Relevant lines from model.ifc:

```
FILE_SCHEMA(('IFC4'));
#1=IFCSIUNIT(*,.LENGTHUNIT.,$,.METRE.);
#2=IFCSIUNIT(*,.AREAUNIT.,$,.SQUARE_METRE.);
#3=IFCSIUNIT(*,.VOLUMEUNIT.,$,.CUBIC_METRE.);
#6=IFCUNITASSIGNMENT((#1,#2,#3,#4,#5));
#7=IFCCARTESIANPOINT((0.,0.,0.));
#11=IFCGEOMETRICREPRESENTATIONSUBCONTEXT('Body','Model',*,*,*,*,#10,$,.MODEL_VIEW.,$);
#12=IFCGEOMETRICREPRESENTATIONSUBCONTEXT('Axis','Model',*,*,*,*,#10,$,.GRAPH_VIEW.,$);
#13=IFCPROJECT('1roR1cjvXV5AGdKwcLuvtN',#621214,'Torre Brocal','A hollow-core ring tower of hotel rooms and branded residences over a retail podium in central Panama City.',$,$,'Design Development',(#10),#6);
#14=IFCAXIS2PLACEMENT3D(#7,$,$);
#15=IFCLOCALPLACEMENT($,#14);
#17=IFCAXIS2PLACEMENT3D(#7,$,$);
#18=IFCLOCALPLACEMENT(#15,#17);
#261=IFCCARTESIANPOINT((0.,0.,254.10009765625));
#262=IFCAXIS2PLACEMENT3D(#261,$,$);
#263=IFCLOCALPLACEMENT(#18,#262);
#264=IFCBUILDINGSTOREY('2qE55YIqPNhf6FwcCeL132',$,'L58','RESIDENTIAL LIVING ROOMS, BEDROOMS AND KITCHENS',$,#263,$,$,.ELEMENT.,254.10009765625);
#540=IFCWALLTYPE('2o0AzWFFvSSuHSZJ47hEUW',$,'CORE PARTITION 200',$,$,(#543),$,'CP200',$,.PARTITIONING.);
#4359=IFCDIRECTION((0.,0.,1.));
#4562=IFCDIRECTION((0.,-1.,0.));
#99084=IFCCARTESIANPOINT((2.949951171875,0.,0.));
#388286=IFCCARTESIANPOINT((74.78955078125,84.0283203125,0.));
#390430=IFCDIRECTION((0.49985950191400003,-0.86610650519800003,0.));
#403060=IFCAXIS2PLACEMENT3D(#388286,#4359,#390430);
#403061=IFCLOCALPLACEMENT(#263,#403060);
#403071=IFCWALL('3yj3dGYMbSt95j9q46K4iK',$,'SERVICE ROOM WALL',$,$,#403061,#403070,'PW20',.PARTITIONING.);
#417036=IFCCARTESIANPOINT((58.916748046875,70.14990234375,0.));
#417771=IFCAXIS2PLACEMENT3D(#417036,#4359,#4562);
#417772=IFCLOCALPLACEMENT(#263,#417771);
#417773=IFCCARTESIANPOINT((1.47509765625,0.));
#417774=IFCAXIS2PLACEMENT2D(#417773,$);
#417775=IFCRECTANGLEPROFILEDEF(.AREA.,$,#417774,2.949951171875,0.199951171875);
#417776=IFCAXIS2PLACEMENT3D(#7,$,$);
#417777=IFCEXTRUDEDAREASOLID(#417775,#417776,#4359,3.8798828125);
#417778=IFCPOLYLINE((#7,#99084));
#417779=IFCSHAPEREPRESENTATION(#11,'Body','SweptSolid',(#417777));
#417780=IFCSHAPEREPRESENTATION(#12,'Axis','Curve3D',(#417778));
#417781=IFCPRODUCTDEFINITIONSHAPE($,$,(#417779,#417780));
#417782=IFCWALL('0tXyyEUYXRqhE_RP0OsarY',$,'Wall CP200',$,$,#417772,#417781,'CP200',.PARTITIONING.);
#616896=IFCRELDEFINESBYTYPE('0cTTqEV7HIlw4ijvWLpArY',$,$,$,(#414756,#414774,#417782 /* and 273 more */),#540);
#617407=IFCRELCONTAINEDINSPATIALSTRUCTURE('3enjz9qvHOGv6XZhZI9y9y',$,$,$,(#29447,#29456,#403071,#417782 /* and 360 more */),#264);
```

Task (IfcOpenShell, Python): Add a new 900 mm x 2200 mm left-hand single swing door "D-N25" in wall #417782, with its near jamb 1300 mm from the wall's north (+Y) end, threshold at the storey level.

```python
import numpy as np
import ifcopenshell
import ifcopenshell.api.feature
import ifcopenshell.api.geometry
import ifcopenshell.api.root
import ifcopenshell.api.spatial
import ifcopenshell.geom
import ifcopenshell.util.element
import ifcopenshell.util.placement
import ifcopenshell.util.representation
import ifcopenshell.util.shape
import ifcopenshell.util.unit

model = ifcopenshell.open("model.ifc")
unit_scale = ifcopenshell.util.unit.calculate_unit_scale(model)
settings = ifcopenshell.geom.settings()


def volume(element):
    """Net volume in cubic metres, openings subtracted."""
    shape = ifcopenshell.geom.create_shape(settings, element)
    return ifcopenshell.util.shape.get_volume(shape.geometry)


wall = model.by_guid("0tXyyEUYXRqhE_RP0OsarY")
storey = ifcopenshell.util.element.get_container(wall, ifc_class="IfcBuildingStorey")
context = ifcopenshell.util.representation.get_context(model, "Model", "Body", "MODEL_VIEW")
before = volume(wall)

width, height, from_end, sill = 0.9, 2.2, 1.3, 0.0  # metres

# The wall runs along its own X axis, and the end named is its -X end.
wall_shape = ifcopenshell.geom.create_shape(settings, wall)
x, y, z = ifcopenshell.util.shape.get_vertices(wall_shape.geometry).T
start = x.min() + from_end
face, thickness = float(y.min()), float(y.max() - y.min())
wall_matrix = ifcopenshell.util.placement.get_local_placement(wall.ObjectPlacement)
level = ifcopenshell.util.placement.get_local_placement(storey.ObjectPlacement)[2, 3]


def in_wall(x, y):
    """Placement at x, y metres in the wall's axes, at sill height."""
    matrix = wall_matrix.copy()
    matrix[:, 3] = wall_matrix @ np.array([x / unit_scale, y / unit_scale, 0.0, 1.0])
    matrix[2, 3] = level + sill / unit_scale
    return matrix


# Opening: a box that overshoots both wall faces by 50 mm.
opening = ifcopenshell.api.root.create_entity(model, ifc_class="IfcOpeningElement", predefined_type="OPENING")
box = ifcopenshell.api.geometry.add_wall_representation(
    model, context=context, length=width, height=height, thickness=thickness + 0.1
)
ifcopenshell.api.geometry.assign_representation(model, product=opening, representation=box)
ifcopenshell.api.geometry.edit_object_placement(model, product=opening, matrix=in_wall(start, face - 0.05), is_si=False)
ifcopenshell.api.feature.add_feature(model, feature=opening, element=wall)

door = ifcopenshell.api.root.create_entity(model, ifc_class="IfcDoor", name="D-N25", predefined_type="DOOR")
door.OverallWidth, door.OverallHeight = width / unit_scale, height / unit_scale
door.OperationType = "SINGLE_SWING_LEFT"
body = ifcopenshell.api.geometry.add_door_representation(
    model,
    context=context,
    overall_width=door.OverallWidth,
    overall_height=door.OverallHeight,
    operation_type="SINGLE_SWING_LEFT",
    lining_properties={"LiningDepth": thickness / unit_scale, "ThresholdDepth": thickness / unit_scale},
)
ifcopenshell.api.geometry.assign_representation(model, product=door, representation=body)
ifcopenshell.api.spatial.assign_container(model, products=[door], relating_structure=storey)
ifcopenshell.api.feature.add_filling(model, opening=opening, element=door)

# The lining spans the wall, so the door starts at the wall face.
ifcopenshell.api.geometry.edit_object_placement(model, product=door, matrix=in_wall(start, face), is_si=False)

after = volume(wall)

print(f"wall volume {before:.3f} -> {after:.3f} m3")

model.write("model-out.ifc")
```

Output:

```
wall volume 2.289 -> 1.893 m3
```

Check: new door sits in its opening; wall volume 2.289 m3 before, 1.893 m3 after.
